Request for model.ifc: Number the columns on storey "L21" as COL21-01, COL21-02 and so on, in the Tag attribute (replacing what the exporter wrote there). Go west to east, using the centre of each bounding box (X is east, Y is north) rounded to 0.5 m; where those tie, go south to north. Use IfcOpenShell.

First a look at what the model holds.

```python
import ifcopenshell
import ifcopenshell.util.element
import ifcopenshell.util.placement

model = ifcopenshell.open("model.ifc")
print(model.schema)
storey = next(s for s in model.by_type("IfcBuildingStorey") if s.Name == "L21")
columns = [e for e in ifcopenshell.util.element.get_decomposition(storey) if e.is_a("IfcColumn")]
for e in sorted(columns, key=lambda e: e.id()):
    origin = ifcopenshell.util.placement.get_local_placement(e.ObjectPlacement)[:3, 3]
    print(e.id(), e.Tag, e.Name, origin.round(2) + 0.0, sep=" | ")
```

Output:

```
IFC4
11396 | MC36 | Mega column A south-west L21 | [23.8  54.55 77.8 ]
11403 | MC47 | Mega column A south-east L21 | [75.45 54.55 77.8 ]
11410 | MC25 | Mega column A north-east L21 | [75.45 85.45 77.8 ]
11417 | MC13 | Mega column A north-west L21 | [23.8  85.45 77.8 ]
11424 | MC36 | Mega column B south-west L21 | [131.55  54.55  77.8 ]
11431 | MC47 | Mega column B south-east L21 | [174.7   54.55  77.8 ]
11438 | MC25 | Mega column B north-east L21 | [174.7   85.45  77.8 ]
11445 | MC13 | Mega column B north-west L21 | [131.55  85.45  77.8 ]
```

```python
import ifcopenshell
import ifcopenshell.geom
import ifcopenshell.util.element
import ifcopenshell.util.shape

model = ifcopenshell.open("model.ifc")
settings = ifcopenshell.geom.settings()
settings.set("use-world-coords", True)


def centre(element):
    shape = ifcopenshell.geom.create_shape(settings, element)
    return ifcopenshell.util.shape.get_bbox_centroid(shape.geometry)


storey = next(s for s in model.by_type("IfcBuildingStorey") if s.Name == "L21")
columns = [e for e in ifcopenshell.util.element.get_decomposition(storey) if e.is_a("IfcColumn")]

# Insertion points can sit at a corner or the storey origin, so sort by the geometry (in metres).
centres = {e: centre(e) for e in columns}
columns.sort(key=lambda e: (round(centres[e][0] / 0.5), centres[e][1]))

for i, e in enumerate(columns, start=1):
    number = f"COL21-{i:02d}"
    e.Tag = number
    print(e.id(), number)

model.write("model_edited.ifc")
```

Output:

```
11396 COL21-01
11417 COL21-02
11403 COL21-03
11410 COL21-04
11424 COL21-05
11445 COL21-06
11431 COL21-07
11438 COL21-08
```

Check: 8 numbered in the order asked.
